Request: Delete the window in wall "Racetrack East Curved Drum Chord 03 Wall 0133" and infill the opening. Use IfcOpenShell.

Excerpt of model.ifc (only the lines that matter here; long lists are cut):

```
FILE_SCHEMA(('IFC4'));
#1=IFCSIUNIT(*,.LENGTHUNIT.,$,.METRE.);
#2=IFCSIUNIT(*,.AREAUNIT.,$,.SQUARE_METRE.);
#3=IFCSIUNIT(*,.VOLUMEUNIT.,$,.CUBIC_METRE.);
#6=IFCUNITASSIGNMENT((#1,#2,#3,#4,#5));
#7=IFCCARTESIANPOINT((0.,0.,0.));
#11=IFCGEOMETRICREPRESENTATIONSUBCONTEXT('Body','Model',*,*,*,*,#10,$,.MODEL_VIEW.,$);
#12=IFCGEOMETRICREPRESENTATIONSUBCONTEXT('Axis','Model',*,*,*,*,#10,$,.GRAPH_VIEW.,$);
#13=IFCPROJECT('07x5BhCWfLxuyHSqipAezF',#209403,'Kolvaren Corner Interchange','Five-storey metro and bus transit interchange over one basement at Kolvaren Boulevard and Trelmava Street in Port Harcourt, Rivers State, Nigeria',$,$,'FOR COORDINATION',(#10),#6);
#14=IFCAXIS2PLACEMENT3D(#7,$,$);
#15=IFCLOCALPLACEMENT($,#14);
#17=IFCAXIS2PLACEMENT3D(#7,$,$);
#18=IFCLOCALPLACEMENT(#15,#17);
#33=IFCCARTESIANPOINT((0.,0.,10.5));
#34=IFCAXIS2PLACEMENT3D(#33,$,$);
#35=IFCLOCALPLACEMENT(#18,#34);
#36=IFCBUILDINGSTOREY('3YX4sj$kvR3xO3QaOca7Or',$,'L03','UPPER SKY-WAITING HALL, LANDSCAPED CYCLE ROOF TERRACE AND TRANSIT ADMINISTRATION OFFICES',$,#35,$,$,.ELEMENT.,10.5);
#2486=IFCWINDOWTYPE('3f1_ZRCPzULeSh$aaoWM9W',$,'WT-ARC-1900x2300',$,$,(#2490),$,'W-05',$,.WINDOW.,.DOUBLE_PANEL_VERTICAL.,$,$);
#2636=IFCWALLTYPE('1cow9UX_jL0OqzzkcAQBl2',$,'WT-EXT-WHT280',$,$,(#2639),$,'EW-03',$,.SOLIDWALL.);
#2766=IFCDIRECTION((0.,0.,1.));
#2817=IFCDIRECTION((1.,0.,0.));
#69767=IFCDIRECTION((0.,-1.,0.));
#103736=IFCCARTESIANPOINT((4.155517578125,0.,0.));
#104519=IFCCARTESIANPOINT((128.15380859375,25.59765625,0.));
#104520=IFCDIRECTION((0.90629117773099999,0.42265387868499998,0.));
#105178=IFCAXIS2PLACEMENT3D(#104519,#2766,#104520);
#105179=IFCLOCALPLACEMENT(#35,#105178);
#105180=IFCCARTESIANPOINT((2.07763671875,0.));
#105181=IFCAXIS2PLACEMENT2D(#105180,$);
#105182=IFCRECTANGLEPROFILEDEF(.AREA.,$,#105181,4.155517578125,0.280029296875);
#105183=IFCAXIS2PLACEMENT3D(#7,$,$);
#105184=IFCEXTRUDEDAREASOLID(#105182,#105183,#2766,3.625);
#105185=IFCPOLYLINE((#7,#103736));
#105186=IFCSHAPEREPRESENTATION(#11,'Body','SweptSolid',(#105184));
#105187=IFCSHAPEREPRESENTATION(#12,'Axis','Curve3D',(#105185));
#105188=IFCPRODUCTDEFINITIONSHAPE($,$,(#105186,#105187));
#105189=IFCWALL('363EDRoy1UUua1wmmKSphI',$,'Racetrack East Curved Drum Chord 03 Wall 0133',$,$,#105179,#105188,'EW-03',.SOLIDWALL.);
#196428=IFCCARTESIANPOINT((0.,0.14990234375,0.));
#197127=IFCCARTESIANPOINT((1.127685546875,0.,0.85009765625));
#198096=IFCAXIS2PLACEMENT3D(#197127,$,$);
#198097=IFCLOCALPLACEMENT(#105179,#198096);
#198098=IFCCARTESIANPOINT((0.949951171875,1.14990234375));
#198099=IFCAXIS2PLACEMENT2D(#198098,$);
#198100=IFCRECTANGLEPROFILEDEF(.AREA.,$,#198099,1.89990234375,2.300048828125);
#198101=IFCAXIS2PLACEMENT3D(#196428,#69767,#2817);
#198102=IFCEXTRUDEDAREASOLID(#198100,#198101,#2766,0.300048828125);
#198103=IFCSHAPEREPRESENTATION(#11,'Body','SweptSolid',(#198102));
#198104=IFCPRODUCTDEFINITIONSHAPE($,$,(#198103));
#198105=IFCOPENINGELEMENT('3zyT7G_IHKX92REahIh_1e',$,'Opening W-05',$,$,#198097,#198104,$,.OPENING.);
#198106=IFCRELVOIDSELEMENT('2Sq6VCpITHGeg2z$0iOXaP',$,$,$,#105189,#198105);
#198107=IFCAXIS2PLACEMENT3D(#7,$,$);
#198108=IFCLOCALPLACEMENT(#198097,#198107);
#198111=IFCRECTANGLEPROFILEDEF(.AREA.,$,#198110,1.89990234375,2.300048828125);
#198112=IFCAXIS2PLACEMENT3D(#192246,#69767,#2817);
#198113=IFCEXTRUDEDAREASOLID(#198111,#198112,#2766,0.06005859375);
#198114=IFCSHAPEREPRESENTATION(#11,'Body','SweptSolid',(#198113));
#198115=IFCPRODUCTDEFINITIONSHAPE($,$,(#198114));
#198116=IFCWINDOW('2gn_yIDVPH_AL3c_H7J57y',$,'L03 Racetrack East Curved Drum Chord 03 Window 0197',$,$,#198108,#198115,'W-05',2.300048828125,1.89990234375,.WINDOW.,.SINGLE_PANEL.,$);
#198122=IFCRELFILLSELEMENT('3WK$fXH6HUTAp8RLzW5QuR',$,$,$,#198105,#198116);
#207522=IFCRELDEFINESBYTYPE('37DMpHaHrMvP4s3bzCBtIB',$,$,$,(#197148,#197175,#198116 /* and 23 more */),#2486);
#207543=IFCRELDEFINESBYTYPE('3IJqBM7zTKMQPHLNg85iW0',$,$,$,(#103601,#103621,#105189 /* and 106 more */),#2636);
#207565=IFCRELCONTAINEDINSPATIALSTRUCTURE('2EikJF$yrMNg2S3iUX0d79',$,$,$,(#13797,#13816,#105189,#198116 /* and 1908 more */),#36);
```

```python
import ifcopenshell
import ifcopenshell.api.feature
import ifcopenshell.api.root
import ifcopenshell.geom
import ifcopenshell.util.shape

model = ifcopenshell.open("model.ifc")
settings = ifcopenshell.geom.settings()


def volume(element):
    """Net volume in cubic metres, openings subtracted."""
    shape = ifcopenshell.geom.create_shape(settings, element)
    return ifcopenshell.util.shape.get_volume(shape.geometry)


window = model.by_guid("2gn_yIDVPH_AL3c_H7J57y")
opening = window.FillsVoids[0].RelatingOpeningElement
wall = opening.VoidsElements[0].RelatingBuildingElement
before = volume(wall)

ifcopenshell.api.root.remove_product(model, product=window)
ifcopenshell.api.feature.remove_feature(model, feature=opening)

after = volume(wall)

print(f"wall volume {before:.3f} -> {after:.3f} m3")

model.write("model_edited.ifc")
```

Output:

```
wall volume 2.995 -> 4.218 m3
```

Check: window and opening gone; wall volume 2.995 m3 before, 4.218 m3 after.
